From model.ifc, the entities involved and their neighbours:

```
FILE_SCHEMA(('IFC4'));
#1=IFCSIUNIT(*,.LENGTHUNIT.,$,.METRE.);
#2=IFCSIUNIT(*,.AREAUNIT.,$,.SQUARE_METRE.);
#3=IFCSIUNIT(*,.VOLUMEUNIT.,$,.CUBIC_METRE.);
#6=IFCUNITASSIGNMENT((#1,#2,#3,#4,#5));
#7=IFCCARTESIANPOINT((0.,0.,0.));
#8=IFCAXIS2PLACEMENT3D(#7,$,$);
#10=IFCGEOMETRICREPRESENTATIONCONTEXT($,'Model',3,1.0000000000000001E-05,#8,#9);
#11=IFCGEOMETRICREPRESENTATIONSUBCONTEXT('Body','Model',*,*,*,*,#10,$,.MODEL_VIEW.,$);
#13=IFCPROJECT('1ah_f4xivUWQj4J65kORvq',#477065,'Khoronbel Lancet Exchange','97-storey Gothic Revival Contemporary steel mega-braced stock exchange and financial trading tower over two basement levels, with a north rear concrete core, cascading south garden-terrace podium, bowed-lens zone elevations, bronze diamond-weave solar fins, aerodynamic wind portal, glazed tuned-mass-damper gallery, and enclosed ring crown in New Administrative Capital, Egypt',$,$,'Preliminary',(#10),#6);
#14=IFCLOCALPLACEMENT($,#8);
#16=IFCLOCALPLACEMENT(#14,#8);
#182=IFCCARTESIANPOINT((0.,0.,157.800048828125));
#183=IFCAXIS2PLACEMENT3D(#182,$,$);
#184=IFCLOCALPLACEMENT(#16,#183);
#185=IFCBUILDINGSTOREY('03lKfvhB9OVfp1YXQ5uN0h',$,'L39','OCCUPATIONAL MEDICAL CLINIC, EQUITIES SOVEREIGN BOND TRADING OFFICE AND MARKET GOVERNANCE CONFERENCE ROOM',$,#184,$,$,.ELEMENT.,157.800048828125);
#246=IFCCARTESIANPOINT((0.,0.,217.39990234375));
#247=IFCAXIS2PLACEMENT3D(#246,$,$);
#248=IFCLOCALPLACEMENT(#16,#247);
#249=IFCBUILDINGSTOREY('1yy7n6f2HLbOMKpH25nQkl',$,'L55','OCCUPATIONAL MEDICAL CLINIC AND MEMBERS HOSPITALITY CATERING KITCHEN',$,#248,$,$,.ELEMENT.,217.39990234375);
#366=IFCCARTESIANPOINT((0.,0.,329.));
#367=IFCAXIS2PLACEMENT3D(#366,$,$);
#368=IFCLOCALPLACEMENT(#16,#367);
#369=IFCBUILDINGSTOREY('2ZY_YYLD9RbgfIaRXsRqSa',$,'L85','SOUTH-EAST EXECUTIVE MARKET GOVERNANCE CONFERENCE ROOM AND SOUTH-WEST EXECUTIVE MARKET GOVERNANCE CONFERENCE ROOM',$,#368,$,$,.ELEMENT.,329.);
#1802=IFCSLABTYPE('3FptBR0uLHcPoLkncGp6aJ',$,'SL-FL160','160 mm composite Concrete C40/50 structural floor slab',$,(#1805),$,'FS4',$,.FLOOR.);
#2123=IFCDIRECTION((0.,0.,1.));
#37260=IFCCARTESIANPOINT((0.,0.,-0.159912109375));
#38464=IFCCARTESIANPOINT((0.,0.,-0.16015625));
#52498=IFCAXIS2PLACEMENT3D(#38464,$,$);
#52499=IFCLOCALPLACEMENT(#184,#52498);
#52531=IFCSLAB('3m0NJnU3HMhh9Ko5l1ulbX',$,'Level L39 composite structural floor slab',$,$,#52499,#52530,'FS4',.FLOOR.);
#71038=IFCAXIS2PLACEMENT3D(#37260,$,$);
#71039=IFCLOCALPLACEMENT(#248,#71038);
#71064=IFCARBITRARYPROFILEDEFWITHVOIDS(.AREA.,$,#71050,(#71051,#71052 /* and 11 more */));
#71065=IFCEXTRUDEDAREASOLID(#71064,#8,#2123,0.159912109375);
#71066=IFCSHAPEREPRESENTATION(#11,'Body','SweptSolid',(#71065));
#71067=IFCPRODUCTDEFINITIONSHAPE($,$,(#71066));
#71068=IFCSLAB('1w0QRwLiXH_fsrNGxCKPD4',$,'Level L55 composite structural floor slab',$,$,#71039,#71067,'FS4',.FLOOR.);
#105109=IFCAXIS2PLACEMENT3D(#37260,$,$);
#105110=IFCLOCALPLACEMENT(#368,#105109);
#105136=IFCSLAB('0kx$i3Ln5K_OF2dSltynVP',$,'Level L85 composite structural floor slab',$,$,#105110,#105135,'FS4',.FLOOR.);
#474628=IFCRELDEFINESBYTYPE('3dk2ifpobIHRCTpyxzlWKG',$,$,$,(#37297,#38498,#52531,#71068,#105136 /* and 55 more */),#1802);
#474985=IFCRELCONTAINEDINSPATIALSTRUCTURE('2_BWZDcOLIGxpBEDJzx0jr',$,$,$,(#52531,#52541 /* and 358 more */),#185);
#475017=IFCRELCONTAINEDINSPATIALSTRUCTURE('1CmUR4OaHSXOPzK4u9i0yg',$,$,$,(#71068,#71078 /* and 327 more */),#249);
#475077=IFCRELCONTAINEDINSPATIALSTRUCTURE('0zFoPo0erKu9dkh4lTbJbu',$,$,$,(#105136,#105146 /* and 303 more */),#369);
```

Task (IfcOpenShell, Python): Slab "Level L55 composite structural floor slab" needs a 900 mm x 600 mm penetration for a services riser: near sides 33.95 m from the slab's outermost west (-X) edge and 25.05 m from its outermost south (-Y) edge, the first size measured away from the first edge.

```python
import numpy as np
import ifcopenshell
import ifcopenshell.api.feature
import ifcopenshell.api.geometry
import ifcopenshell.api.root
import ifcopenshell.geom
import ifcopenshell.util.placement
import ifcopenshell.util.representation
import ifcopenshell.util.shape
import ifcopenshell.util.unit

model = ifcopenshell.open("model.ifc")
unit_scale = ifcopenshell.util.unit.calculate_unit_scale(model)
settings = ifcopenshell.geom.settings()


def volume(element):
    """Net volume in cubic metres, openings subtracted."""
    shape = ifcopenshell.geom.create_shape(settings, element)
    return ifcopenshell.util.shape.get_volume(shape.geometry)


slab = model.by_guid("1w0QRwLiXH_fsrNGxCKPD4")
before = volume(slab)

# Extent in the slab's own axes, in metres. The edges named are its -X and -Y sides.
slab_shape = ifcopenshell.geom.create_shape(settings, slab)
vertices = ifcopenshell.util.shape.get_vertices(slab_shape.geometry)
x_min, y_min, bottom = vertices.min(axis=0)
top = vertices[:, 2].max()

opening = ifcopenshell.api.root.create_entity(model, ifc_class="IfcOpeningElement", name="Services riser opening", predefined_type="OPENING")
context = ifcopenshell.util.representation.get_context(model, "Model", "Body", "MODEL_VIEW")
width, depth = 0.9, 0.6
outline = [(0.0, 0.0), (width, 0.0), (width, depth), (0.0, depth), (0.0, 0.0)]
# Overshoot both faces by 50 mm so the cut is clean.
shape = ifcopenshell.api.geometry.add_slab_representation(
    model, context=context, depth=top - bottom + 0.1, polyline=outline
)
ifcopenshell.api.geometry.assign_representation(model, product=opening, representation=shape)

matrix = ifcopenshell.util.placement.get_local_placement(slab.ObjectPlacement)
matrix[:, 3] = matrix @ np.append(np.array([x_min + 33.95, y_min + 25.05, bottom - 0.05]) / unit_scale, 1.0)
ifcopenshell.api.geometry.edit_object_placement(model, product=opening, matrix=matrix, is_si=False)
ifcopenshell.api.feature.add_feature(model, feature=opening, element=slab)

after = volume(slab)

print(f"slab volume {before:.3f} -> {after:.3f} m3")

model.write("model_updated.ifc")
```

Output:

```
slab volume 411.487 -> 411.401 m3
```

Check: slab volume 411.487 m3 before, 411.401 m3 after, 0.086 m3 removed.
